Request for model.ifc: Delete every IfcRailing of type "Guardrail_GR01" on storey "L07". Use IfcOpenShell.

First a look at what the model holds.

```python
import ifcopenshell
import ifcopenshell.util.element

model = ifcopenshell.open("model.ifc")
print(model.schema)
storey = next(s for s in model.by_type("IfcBuildingStorey") if s.Name == "L07")
railings = [e for e in ifcopenshell.util.element.get_decomposition(storey) if e.is_a("IfcRailing")]
seen = {}
for e in railings:
    element_type = ifcopenshell.util.element.get_type(e)
    name = element_type.Name if element_type not in (None, e) else None
    seen[name] = seen.get(name, 0) + 1
for name, count in sorted(seen.items(), key=str):
    print(count, "x", name)
```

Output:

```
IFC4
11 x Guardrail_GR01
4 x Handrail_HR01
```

```python
import ifcopenshell
import ifcopenshell.api.root
import ifcopenshell.util.element

model = ifcopenshell.open("model.ifc")

storey = next(s for s in model.by_type("IfcBuildingStorey") if s.Name == "L07")
railings = [e for e in ifcopenshell.util.element.get_decomposition(storey) if e.is_a("IfcRailing")]
targets = [e for e in railings if (t := ifcopenshell.util.element.get_type(e)) not in (None, e) and t.Name == "Guardrail_GR01"]

for e in targets:
    ifcopenshell.api.root.remove_product(model, product=e)
print(len(targets), "removed")

model.write("model-out.ifc")
```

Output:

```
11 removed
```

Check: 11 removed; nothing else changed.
